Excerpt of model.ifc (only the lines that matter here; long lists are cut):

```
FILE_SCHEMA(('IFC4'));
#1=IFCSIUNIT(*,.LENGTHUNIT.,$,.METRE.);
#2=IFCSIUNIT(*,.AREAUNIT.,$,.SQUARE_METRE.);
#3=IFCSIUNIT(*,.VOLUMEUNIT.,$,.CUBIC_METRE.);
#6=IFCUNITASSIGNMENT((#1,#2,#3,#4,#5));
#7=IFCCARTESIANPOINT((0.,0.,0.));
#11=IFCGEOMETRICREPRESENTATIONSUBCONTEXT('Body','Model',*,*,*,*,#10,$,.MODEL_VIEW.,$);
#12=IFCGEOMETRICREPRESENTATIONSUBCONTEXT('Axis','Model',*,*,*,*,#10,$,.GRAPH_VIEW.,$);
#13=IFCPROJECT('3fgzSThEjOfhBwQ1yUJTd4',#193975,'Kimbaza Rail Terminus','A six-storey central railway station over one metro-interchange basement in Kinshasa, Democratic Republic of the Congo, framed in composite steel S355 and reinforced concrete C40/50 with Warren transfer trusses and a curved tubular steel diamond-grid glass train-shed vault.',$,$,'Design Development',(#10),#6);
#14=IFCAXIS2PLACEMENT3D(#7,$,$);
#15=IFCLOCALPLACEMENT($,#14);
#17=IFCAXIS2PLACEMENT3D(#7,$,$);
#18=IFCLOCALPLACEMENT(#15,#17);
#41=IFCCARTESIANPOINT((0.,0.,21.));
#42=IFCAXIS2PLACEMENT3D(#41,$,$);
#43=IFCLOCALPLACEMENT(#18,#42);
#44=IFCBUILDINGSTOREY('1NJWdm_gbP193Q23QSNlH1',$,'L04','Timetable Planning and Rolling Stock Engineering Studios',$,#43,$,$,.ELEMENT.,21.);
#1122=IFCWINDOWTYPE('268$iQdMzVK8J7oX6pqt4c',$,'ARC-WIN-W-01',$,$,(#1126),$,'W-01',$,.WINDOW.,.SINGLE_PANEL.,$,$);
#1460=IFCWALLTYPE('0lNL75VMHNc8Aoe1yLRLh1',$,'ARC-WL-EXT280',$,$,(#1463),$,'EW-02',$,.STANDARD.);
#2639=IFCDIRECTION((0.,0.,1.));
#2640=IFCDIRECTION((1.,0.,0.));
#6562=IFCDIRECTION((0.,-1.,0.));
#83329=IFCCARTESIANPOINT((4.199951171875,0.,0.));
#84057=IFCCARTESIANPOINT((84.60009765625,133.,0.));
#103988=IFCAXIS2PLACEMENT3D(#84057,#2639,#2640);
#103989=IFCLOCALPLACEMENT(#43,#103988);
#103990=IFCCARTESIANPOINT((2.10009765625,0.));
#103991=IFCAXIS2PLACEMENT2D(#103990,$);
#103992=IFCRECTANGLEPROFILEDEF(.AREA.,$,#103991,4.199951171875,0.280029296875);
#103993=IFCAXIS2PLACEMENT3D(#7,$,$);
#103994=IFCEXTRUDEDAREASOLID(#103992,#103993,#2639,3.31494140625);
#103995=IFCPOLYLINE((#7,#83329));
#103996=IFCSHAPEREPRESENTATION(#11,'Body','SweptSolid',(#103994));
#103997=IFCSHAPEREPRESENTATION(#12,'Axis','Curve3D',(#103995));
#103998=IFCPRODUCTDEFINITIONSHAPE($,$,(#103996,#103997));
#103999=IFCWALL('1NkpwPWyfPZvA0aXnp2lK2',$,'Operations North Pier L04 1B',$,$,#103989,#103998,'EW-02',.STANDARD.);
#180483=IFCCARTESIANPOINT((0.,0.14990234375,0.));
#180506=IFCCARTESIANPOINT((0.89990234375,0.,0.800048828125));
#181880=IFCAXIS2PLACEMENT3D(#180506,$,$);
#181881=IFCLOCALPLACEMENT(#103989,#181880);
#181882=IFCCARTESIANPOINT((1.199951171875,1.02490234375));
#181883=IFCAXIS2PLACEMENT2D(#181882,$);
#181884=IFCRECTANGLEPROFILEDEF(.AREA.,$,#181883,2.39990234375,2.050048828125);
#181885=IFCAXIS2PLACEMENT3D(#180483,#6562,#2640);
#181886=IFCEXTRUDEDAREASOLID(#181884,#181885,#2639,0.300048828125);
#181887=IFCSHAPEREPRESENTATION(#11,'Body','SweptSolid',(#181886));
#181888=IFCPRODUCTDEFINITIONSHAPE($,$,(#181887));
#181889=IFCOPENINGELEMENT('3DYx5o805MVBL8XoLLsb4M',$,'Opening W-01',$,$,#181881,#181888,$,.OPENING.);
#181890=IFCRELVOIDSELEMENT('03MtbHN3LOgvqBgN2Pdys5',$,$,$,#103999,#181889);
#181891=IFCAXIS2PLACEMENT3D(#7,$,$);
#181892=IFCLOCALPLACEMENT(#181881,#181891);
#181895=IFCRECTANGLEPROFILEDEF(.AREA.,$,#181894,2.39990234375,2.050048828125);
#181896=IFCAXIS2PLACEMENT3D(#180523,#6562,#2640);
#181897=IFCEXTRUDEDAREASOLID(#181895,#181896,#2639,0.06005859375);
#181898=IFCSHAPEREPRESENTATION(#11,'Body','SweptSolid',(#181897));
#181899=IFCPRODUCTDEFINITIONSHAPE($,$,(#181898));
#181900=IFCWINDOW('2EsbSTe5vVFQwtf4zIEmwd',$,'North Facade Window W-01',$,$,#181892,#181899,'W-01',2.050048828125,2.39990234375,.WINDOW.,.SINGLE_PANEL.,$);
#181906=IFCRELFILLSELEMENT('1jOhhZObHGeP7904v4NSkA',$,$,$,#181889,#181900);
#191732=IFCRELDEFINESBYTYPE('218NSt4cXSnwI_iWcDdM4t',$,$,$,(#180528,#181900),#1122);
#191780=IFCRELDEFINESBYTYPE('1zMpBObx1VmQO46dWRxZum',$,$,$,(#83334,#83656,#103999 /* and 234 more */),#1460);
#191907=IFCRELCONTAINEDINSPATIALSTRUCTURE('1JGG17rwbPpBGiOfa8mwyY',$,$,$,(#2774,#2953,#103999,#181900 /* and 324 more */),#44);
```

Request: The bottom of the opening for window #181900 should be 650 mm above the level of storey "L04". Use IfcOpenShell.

```python
import numpy as np
import ifcopenshell
import ifcopenshell.api.geometry
import ifcopenshell.geom
import ifcopenshell.util.element
import ifcopenshell.util.placement
import ifcopenshell.util.shape
import ifcopenshell.util.unit

model = ifcopenshell.open("model.ifc")
unit_scale = ifcopenshell.util.unit.calculate_unit_scale(model)

window = model.by_guid("2EsbSTe5vVFQwtf4zIEmwd")
opening = window.FillsVoids[0].RelatingOpeningElement
storey = ifcopenshell.util.element.get_container(window, ifc_class="IfcBuildingStorey")
level = ifcopenshell.util.placement.get_local_placement(storey.ObjectPlacement)[2, 3]

# The opening's origin need not be at the sill, so measure its lowest point.
shape = ifcopenshell.geom.create_shape(ifcopenshell.geom.settings(), opening)
bottom = ifcopenshell.util.shape.get_shape_bottom_elevation(shape, shape.geometry) / unit_scale
dz = level + 0.65 - bottom

shift = np.array([0.0, 0.0, dz])
# The window is placed relative to its opening, so it follows when the opening moves.
matrix = ifcopenshell.util.placement.get_local_placement(opening.ObjectPlacement)
matrix[:3, 3] += shift
ifcopenshell.api.geometry.edit_object_placement(
    model, product=opening, matrix=matrix, is_si=False, should_transform_children=True
)

print(f"moved by {dz * unit_scale:+.3f} m")

model.write("model_edited.ifc")
```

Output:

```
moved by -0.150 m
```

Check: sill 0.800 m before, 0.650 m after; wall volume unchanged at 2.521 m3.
